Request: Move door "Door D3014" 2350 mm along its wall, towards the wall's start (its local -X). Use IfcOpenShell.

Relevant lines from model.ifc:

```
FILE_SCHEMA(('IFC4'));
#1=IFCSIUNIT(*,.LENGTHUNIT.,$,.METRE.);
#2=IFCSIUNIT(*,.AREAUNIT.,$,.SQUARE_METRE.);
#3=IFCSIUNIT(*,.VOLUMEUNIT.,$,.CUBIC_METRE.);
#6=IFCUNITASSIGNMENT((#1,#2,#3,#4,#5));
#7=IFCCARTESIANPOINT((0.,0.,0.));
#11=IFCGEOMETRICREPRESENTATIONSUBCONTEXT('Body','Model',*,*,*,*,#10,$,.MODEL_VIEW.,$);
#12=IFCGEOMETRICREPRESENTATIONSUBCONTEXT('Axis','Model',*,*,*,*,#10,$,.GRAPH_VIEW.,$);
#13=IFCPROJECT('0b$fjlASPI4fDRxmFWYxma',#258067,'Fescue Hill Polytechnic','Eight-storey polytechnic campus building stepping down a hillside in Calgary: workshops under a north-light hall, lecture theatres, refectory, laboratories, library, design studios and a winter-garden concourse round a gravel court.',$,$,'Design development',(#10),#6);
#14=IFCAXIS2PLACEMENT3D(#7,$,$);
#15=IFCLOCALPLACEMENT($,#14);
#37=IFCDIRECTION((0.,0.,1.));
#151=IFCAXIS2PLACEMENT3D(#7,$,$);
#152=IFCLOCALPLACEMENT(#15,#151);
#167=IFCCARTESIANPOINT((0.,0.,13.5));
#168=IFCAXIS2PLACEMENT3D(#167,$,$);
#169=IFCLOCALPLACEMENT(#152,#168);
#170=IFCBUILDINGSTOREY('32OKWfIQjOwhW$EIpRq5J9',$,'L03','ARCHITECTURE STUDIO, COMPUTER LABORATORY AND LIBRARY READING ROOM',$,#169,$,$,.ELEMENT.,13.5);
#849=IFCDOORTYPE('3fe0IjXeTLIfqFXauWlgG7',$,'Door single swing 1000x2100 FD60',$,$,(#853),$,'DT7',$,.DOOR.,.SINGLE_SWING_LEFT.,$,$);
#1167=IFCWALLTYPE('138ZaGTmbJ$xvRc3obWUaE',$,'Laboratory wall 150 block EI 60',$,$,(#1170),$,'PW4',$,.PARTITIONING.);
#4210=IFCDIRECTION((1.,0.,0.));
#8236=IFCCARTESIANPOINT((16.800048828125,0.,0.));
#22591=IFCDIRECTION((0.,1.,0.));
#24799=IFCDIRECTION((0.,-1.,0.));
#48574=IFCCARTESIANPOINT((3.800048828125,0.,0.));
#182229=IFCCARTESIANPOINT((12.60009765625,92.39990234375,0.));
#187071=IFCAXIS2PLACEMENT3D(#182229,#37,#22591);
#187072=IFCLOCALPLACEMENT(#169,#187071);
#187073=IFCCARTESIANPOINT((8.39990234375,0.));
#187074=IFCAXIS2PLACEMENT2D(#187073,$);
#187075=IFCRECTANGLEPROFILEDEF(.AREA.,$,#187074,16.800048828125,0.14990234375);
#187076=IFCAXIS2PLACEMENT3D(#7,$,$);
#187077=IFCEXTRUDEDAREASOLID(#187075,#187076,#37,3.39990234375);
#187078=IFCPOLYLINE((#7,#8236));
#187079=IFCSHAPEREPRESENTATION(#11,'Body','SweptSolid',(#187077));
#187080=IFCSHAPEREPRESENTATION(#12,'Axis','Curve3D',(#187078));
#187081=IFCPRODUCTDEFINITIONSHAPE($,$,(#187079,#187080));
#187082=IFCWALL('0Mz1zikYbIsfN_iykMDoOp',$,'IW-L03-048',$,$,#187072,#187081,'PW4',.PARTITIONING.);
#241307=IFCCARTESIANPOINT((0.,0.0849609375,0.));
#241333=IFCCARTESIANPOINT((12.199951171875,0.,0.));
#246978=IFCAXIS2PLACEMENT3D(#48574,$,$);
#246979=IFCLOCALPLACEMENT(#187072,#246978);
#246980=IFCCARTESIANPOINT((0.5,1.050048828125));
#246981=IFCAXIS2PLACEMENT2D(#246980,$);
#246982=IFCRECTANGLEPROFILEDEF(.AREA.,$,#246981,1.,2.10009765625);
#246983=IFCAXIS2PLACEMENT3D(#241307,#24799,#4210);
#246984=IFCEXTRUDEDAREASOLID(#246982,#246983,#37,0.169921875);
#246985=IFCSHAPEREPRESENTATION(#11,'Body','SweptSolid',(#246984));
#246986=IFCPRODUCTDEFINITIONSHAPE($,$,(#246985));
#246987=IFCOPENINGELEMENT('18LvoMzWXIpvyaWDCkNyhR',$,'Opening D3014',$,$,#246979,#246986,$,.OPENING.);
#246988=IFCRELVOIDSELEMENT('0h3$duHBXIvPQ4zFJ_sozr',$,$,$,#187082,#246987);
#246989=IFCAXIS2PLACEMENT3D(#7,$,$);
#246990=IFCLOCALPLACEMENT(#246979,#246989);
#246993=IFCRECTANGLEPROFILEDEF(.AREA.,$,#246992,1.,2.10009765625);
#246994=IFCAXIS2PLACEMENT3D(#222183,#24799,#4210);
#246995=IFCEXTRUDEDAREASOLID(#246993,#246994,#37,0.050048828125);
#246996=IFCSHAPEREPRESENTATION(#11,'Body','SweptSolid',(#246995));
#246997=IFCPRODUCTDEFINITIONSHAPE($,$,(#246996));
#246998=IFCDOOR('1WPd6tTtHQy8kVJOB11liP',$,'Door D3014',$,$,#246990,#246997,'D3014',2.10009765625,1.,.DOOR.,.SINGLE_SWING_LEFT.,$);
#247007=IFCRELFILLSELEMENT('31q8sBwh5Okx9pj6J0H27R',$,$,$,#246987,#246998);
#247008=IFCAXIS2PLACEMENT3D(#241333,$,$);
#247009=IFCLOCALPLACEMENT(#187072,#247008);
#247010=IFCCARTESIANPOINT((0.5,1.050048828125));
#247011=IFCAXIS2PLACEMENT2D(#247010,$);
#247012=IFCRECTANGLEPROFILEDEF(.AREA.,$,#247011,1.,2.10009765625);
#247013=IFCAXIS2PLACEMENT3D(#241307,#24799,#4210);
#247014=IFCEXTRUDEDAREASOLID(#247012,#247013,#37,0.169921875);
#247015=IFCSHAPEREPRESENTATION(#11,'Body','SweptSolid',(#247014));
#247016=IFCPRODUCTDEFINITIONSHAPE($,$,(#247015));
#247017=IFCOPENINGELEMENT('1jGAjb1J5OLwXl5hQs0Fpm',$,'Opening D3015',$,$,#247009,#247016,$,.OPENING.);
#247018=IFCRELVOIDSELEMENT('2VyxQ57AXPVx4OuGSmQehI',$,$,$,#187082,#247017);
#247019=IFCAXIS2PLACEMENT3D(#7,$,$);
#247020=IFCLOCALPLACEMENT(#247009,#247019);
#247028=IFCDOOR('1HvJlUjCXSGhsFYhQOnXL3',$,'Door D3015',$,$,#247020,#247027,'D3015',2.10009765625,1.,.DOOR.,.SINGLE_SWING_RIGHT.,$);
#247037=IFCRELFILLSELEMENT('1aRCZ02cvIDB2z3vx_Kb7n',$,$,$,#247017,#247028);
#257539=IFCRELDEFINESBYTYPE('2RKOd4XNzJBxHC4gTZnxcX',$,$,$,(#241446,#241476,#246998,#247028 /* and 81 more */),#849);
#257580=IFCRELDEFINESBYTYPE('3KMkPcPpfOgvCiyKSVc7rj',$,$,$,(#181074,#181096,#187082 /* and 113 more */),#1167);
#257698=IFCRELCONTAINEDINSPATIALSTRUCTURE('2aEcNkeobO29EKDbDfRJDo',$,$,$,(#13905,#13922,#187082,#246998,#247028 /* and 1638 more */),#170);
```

```python
import ifcopenshell
import ifcopenshell.api.geometry
import ifcopenshell.util.placement
import ifcopenshell.util.unit

model = ifcopenshell.open("model.ifc")
unit_scale = ifcopenshell.util.unit.calculate_unit_scale(model)

door = model.by_guid("1WPd6tTtHQy8kVJOB11liP")
opening = door.FillsVoids[0].RelatingOpeningElement
wall = opening.VoidsElements[0].RelatingBuildingElement

wall_matrix = ifcopenshell.util.placement.get_local_placement(wall.ObjectPlacement)
shift = wall_matrix[:3, 0] * -2.35 / unit_scale
before = ifcopenshell.util.placement.get_local_placement(door.ObjectPlacement)[:3, 3].copy()

# The door is placed relative to its opening, so it follows when the opening moves.
matrix = ifcopenshell.util.placement.get_local_placement(opening.ObjectPlacement)
matrix[:3, 3] += shift
ifcopenshell.api.geometry.edit_object_placement(
    model, product=opening, matrix=matrix, is_si=False, should_transform_children=True
)

after = ifcopenshell.util.placement.get_local_placement(door.ObjectPlacement)[:3, 3]
print("door moved by", (after - before).round(3) + 0.0)

model.write("model_updated.ifc")
```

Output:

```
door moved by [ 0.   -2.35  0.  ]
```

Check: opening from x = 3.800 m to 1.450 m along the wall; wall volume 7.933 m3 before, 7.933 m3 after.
